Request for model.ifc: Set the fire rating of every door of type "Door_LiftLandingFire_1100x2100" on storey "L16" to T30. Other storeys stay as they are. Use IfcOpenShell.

First a look at what the model holds.

```python
import ifcopenshell
import ifcopenshell.util.element

model = ifcopenshell.open("model.ifc")
print(model.schema)
storey = next(s for s in model.by_type("IfcBuildingStorey") if s.Name == "L16")
doors = [e for e in ifcopenshell.util.element.get_decomposition(storey) if e.is_a("IfcDoor")]
seen = {}
for e in doors:
    element_type = ifcopenshell.util.element.get_type(e)
    key = (element_type.Name if element_type != e and element_type else None, ifcopenshell.util.element.get_pset(e, "Pset_DoorCommon", "FireRating"))
    seen[key] = seen.get(key, 0) + 1
for (name, value), count in sorted(seen.items(), key=str):
    print(count, "x", name, "|", value)
```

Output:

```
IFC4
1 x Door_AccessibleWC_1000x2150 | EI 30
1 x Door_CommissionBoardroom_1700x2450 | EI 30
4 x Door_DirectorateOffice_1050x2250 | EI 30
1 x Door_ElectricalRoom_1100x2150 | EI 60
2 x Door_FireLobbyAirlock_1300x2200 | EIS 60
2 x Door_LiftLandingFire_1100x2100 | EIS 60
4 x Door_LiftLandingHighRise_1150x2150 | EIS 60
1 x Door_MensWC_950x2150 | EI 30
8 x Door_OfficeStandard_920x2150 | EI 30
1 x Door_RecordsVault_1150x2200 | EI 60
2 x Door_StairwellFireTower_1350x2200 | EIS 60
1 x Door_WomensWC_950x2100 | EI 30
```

```python
import ifcopenshell
import ifcopenshell.api.pset
import ifcopenshell.util.element

model = ifcopenshell.open("model.ifc")

storey = next(s for s in model.by_type("IfcBuildingStorey") if s.Name == "L16")
doors = [e for e in ifcopenshell.util.element.get_decomposition(storey) if e.is_a("IfcDoor")]

count = 0
for e in doors:
    element_type = ifcopenshell.util.element.get_type(e)
    if element_type in (None, e) or element_type.Name != "Door_LiftLandingFire_1100x2100":
        continue
    # add_pset returns the element's existing set when there is one.
    pset = ifcopenshell.api.pset.add_pset(model, product=e, name="Pset_DoorCommon")
    ifcopenshell.api.pset.edit_pset(model, pset=pset, properties={"FireRating": "T30"})
    count += 1

print(count, "doors updated")

model.write("model_v2.ifc")
```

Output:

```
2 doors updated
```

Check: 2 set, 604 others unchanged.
